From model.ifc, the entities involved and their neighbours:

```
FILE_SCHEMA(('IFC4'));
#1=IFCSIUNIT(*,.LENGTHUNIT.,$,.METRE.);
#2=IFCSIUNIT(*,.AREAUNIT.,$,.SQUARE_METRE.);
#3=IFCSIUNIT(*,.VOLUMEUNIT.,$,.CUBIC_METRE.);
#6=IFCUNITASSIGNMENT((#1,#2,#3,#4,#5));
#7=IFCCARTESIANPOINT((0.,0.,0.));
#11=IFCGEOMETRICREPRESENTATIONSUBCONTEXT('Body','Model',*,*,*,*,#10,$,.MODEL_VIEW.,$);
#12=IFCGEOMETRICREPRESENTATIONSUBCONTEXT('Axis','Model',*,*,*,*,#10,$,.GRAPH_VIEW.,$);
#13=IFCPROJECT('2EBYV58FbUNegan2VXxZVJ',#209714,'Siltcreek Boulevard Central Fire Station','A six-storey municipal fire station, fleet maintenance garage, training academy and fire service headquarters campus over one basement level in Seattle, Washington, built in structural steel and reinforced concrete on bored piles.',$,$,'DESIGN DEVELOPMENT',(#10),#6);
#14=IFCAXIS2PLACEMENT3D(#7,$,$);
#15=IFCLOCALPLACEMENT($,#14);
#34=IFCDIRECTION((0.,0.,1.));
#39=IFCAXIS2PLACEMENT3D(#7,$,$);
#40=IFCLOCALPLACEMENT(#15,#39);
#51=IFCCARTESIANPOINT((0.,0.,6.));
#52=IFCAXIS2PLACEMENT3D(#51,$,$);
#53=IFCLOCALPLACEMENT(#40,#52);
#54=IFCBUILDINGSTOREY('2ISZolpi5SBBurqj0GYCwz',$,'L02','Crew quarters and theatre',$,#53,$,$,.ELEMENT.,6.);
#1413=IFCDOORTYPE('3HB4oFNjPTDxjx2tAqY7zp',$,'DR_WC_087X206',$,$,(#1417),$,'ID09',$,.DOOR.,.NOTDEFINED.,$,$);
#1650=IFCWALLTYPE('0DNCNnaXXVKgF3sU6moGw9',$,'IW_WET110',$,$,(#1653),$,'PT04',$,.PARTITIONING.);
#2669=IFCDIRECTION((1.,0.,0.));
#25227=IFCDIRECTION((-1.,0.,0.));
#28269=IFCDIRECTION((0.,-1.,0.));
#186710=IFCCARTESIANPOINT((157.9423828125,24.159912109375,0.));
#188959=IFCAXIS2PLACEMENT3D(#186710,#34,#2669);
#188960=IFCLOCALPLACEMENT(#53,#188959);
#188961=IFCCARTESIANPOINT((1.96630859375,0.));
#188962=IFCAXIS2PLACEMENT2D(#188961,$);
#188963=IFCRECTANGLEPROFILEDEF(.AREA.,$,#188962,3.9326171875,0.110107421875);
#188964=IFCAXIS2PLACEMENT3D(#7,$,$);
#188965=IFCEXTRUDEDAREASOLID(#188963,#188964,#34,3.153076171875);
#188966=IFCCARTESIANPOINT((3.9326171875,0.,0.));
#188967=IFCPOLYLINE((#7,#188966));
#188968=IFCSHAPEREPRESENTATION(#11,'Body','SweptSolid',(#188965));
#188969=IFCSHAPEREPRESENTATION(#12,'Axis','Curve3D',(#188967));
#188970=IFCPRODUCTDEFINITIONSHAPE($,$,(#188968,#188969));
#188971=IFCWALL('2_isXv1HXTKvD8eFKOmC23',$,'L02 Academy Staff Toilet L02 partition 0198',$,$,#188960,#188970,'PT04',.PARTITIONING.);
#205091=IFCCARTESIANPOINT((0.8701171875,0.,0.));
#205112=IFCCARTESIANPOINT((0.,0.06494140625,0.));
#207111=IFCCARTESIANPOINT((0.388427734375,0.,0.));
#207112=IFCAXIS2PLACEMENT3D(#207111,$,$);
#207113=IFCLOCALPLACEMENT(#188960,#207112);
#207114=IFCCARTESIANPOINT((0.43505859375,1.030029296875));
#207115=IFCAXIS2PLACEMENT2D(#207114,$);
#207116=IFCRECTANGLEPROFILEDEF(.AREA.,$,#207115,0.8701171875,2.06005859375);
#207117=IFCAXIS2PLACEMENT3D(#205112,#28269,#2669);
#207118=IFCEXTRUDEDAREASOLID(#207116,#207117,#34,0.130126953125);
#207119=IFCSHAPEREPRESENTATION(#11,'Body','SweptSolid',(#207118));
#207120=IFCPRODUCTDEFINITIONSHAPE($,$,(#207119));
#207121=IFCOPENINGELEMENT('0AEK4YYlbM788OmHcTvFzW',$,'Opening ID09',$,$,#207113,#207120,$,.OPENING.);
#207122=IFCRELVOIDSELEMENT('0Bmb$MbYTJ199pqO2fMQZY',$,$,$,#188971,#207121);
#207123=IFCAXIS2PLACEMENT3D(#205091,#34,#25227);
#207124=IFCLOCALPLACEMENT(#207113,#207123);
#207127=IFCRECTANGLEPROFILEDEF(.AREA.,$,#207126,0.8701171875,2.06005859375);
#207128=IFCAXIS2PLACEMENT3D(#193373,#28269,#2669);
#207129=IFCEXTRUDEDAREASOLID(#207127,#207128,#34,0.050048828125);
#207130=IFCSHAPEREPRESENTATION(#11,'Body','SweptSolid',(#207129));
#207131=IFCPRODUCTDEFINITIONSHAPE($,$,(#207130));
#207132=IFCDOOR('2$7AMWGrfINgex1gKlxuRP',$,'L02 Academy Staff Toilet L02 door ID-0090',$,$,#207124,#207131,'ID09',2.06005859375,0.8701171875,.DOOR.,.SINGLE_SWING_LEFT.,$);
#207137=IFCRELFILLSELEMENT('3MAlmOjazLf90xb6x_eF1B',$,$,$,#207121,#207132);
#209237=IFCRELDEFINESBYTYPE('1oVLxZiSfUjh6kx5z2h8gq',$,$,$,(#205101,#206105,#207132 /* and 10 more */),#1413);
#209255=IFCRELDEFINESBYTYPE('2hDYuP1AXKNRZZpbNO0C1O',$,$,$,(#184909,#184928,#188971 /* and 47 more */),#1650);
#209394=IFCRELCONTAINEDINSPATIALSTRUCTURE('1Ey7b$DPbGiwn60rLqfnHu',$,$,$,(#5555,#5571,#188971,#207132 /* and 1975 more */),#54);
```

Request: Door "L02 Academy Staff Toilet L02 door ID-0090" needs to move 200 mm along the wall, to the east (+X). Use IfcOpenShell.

```python
import ifcopenshell
import ifcopenshell.api.geometry
import ifcopenshell.util.placement

model = ifcopenshell.open("model.ifc")

door = model.by_guid("2$7AMWGrfINgex1gKlxuRP")
opening = door.FillsVoids[0].RelatingOpeningElement
wall = opening.VoidsElements[0].RelatingBuildingElement

wall_matrix = ifcopenshell.util.placement.get_local_placement(wall.ObjectPlacement)
shift = wall_matrix[:3, 0] * 0.2
before = ifcopenshell.util.placement.get_local_placement(door.ObjectPlacement)[:3, 3].copy()

# The door is placed relative to its opening, so it follows when the opening moves.
matrix = ifcopenshell.util.placement.get_local_placement(opening.ObjectPlacement)
matrix[:3, 3] += shift
ifcopenshell.api.geometry.edit_object_placement(
    model, product=opening, matrix=matrix, is_si=False, should_transform_children=True
)

after = ifcopenshell.util.placement.get_local_placement(door.ObjectPlacement)[:3, 3]
print("door moved by", (after - before).round(3) + 0.0)

model.write("model_edited.ifc")
```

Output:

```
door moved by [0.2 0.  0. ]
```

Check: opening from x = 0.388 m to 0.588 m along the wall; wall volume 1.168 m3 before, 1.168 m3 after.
